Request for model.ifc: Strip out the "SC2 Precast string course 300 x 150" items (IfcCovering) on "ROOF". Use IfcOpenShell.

First a look at what the model holds.

```python
import ifcopenshell
import ifcopenshell.util.element

model = ifcopenshell.open("model.ifc")
print(model.schema)
storey = next(s for s in model.by_type("IfcBuildingStorey") if s.Name == "ROOF")
coverings = [e for e in ifcopenshell.util.element.get_decomposition(storey) if e.is_a("IfcCovering")]
seen = {}
for e in coverings:
    element_type = ifcopenshell.util.element.get_type(e)
    name = element_type.Name if element_type not in (None, e) else None
    seen[name] = seen.get(name, 0) + 1
for name, count in sorted(seen.items(), key=str):
    print(count, "x", name)
```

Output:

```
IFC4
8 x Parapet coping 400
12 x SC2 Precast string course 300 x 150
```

```python
import ifcopenshell
import ifcopenshell.api.root
import ifcopenshell.util.element

model = ifcopenshell.open("model.ifc")

storey = next(s for s in model.by_type("IfcBuildingStorey") if s.Name == "ROOF")
coverings = [e for e in ifcopenshell.util.element.get_decomposition(storey) if e.is_a("IfcCovering")]
targets = [e for e in coverings if (t := ifcopenshell.util.element.get_type(e)) not in (None, e) and t.Name == "SC2 Precast string course 300 x 150"]

for e in targets:
    ifcopenshell.api.root.remove_product(model, product=e)
print(len(targets), "removed")

model.write("model_v2.ifc")
```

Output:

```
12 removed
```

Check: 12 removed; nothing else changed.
